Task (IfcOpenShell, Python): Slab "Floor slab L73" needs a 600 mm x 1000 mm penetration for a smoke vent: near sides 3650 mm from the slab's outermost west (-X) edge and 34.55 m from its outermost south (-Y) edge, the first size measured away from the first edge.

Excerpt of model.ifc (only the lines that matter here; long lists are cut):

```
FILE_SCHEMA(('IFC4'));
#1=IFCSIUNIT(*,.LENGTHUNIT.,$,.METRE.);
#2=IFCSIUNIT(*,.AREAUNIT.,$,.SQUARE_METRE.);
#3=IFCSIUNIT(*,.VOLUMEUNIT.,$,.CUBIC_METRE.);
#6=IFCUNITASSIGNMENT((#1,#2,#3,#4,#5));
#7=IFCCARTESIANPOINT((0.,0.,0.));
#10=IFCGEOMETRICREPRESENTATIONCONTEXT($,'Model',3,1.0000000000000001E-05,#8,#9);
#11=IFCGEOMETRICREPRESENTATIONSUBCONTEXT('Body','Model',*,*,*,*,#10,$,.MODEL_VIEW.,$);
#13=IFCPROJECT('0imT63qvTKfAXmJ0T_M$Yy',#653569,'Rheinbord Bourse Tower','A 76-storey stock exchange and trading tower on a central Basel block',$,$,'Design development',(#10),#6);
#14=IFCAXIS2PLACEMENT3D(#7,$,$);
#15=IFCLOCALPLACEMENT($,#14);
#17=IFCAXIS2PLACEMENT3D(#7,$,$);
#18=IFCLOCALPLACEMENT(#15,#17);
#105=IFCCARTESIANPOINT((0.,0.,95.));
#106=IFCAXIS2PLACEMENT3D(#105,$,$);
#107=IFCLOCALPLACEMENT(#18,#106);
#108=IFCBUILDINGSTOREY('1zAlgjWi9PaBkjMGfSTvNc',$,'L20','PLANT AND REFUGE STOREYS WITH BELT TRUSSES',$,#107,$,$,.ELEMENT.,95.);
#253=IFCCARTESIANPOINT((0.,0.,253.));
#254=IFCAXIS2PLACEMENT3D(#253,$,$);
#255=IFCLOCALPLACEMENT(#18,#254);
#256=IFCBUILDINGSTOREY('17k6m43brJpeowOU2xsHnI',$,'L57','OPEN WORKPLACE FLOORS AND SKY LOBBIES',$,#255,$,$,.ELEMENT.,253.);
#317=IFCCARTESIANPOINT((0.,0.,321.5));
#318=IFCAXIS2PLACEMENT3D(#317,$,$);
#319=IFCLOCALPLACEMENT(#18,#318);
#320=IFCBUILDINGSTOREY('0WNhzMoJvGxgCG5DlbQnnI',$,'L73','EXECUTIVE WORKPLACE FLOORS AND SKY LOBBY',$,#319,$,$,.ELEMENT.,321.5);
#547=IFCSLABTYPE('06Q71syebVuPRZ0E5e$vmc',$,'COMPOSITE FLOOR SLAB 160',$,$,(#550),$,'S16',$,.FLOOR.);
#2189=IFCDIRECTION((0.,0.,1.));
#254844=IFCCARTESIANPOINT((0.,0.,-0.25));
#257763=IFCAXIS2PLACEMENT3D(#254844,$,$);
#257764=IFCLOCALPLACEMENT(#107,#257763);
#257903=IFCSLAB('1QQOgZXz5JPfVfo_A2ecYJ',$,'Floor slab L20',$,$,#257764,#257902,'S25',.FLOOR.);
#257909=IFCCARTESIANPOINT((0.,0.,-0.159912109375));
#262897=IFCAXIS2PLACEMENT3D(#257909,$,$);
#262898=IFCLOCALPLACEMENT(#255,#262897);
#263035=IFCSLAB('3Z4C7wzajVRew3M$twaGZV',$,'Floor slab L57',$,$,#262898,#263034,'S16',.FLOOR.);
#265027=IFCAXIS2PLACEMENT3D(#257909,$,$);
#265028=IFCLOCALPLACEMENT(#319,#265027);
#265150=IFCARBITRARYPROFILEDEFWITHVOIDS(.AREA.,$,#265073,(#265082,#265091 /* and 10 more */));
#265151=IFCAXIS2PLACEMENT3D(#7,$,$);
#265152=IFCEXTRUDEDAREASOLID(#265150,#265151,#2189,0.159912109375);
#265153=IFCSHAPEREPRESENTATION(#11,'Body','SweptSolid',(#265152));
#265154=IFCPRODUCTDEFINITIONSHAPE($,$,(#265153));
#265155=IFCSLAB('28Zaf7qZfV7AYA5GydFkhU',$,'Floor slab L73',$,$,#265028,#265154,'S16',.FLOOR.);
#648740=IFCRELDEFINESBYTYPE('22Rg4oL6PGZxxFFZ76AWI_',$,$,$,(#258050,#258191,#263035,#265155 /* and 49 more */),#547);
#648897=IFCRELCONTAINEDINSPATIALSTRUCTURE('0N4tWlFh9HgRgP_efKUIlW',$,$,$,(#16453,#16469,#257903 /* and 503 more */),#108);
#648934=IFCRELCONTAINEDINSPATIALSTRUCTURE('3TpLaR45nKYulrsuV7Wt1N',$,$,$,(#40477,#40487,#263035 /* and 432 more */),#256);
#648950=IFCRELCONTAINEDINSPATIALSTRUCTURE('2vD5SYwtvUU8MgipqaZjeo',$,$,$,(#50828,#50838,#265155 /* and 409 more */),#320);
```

```python
import numpy as np
import ifcopenshell
import ifcopenshell.api.feature
import ifcopenshell.api.geometry
import ifcopenshell.api.root
import ifcopenshell.geom
import ifcopenshell.util.placement
import ifcopenshell.util.representation
import ifcopenshell.util.shape
import ifcopenshell.util.unit

model = ifcopenshell.open("model.ifc")
unit_scale = ifcopenshell.util.unit.calculate_unit_scale(model)
settings = ifcopenshell.geom.settings()


def volume(element):
    """Net volume in cubic metres, openings subtracted."""
    shape = ifcopenshell.geom.create_shape(settings, element)
    return ifcopenshell.util.shape.get_volume(shape.geometry)


slab = model.by_guid("28Zaf7qZfV7AYA5GydFkhU")
before = volume(slab)

# Extent in the slab's own axes, in metres. The edges named are its -X and -Y sides.
slab_shape = ifcopenshell.geom.create_shape(settings, slab)
vertices = ifcopenshell.util.shape.get_vertices(slab_shape.geometry)
x_min, y_min, bottom = vertices.min(axis=0)
top = vertices[:, 2].max()

opening = ifcopenshell.api.root.create_entity(model, ifc_class="IfcOpeningElement", name="Smoke vent opening", predefined_type="OPENING")
context = ifcopenshell.util.representation.get_context(model, "Model", "Body", "MODEL_VIEW")
width, depth = 0.6, 1
outline = [(0.0, 0.0), (width, 0.0), (width, depth), (0.0, depth), (0.0, 0.0)]
# Overshoot both faces by 50 mm so the cut is clean.
shape = ifcopenshell.api.geometry.add_slab_representation(
    model, context=context, depth=top - bottom + 0.1, polyline=outline
)
ifcopenshell.api.geometry.assign_representation(model, product=opening, representation=shape)

matrix = ifcopenshell.util.placement.get_local_placement(slab.ObjectPlacement)
matrix[:, 3] = matrix @ np.append(np.array([x_min + 3.65, y_min + 34.55, bottom - 0.05]) / unit_scale, 1.0)
ifcopenshell.api.geometry.edit_object_placement(model, product=opening, matrix=matrix, is_si=False)
ifcopenshell.api.feature.add_feature(model, feature=opening, element=slab)

after = volume(slab)

print(f"slab volume {before:.3f} -> {after:.3f} m3")

model.write("model_edited.ifc")
```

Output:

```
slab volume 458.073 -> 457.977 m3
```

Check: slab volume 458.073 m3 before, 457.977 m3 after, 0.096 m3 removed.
